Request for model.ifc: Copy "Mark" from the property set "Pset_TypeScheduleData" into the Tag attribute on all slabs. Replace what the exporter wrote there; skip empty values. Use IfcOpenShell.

First a look at what the model holds.

```python
import ifcopenshell
import ifcopenshell.util.element

model = ifcopenshell.open("model.ifc")
print(model.schema)
slabs = model.by_type("IfcSlab")
print(len(slabs), "slabs")
for e in slabs[:8]:
    source = ifcopenshell.util.element.get_pset(e, "Pset_TypeScheduleData", "Mark")
    target = e.Tag
    print(e.id(), repr(source), repr(target), sep=" | ")
```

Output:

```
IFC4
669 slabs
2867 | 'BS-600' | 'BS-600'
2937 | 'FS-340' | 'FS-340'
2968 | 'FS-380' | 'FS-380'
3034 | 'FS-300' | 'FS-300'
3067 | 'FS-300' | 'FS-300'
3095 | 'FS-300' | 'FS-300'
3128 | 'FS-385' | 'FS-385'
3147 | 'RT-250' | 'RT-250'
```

```python
import ifcopenshell
import ifcopenshell.util.element

model = ifcopenshell.open("model.ifc")

count = 0
for e in model.by_type("IfcSlab"):
    value = ifcopenshell.util.element.get_pset(e, "Pset_TypeScheduleData", "Mark")
    current = e.Tag
    if not value or not value.strip() or current == value:
        continue
    e.Tag = value
    count += 1

print(count, "slabs updated")

model.write("model_updated.ifc")
```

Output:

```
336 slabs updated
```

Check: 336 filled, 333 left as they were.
